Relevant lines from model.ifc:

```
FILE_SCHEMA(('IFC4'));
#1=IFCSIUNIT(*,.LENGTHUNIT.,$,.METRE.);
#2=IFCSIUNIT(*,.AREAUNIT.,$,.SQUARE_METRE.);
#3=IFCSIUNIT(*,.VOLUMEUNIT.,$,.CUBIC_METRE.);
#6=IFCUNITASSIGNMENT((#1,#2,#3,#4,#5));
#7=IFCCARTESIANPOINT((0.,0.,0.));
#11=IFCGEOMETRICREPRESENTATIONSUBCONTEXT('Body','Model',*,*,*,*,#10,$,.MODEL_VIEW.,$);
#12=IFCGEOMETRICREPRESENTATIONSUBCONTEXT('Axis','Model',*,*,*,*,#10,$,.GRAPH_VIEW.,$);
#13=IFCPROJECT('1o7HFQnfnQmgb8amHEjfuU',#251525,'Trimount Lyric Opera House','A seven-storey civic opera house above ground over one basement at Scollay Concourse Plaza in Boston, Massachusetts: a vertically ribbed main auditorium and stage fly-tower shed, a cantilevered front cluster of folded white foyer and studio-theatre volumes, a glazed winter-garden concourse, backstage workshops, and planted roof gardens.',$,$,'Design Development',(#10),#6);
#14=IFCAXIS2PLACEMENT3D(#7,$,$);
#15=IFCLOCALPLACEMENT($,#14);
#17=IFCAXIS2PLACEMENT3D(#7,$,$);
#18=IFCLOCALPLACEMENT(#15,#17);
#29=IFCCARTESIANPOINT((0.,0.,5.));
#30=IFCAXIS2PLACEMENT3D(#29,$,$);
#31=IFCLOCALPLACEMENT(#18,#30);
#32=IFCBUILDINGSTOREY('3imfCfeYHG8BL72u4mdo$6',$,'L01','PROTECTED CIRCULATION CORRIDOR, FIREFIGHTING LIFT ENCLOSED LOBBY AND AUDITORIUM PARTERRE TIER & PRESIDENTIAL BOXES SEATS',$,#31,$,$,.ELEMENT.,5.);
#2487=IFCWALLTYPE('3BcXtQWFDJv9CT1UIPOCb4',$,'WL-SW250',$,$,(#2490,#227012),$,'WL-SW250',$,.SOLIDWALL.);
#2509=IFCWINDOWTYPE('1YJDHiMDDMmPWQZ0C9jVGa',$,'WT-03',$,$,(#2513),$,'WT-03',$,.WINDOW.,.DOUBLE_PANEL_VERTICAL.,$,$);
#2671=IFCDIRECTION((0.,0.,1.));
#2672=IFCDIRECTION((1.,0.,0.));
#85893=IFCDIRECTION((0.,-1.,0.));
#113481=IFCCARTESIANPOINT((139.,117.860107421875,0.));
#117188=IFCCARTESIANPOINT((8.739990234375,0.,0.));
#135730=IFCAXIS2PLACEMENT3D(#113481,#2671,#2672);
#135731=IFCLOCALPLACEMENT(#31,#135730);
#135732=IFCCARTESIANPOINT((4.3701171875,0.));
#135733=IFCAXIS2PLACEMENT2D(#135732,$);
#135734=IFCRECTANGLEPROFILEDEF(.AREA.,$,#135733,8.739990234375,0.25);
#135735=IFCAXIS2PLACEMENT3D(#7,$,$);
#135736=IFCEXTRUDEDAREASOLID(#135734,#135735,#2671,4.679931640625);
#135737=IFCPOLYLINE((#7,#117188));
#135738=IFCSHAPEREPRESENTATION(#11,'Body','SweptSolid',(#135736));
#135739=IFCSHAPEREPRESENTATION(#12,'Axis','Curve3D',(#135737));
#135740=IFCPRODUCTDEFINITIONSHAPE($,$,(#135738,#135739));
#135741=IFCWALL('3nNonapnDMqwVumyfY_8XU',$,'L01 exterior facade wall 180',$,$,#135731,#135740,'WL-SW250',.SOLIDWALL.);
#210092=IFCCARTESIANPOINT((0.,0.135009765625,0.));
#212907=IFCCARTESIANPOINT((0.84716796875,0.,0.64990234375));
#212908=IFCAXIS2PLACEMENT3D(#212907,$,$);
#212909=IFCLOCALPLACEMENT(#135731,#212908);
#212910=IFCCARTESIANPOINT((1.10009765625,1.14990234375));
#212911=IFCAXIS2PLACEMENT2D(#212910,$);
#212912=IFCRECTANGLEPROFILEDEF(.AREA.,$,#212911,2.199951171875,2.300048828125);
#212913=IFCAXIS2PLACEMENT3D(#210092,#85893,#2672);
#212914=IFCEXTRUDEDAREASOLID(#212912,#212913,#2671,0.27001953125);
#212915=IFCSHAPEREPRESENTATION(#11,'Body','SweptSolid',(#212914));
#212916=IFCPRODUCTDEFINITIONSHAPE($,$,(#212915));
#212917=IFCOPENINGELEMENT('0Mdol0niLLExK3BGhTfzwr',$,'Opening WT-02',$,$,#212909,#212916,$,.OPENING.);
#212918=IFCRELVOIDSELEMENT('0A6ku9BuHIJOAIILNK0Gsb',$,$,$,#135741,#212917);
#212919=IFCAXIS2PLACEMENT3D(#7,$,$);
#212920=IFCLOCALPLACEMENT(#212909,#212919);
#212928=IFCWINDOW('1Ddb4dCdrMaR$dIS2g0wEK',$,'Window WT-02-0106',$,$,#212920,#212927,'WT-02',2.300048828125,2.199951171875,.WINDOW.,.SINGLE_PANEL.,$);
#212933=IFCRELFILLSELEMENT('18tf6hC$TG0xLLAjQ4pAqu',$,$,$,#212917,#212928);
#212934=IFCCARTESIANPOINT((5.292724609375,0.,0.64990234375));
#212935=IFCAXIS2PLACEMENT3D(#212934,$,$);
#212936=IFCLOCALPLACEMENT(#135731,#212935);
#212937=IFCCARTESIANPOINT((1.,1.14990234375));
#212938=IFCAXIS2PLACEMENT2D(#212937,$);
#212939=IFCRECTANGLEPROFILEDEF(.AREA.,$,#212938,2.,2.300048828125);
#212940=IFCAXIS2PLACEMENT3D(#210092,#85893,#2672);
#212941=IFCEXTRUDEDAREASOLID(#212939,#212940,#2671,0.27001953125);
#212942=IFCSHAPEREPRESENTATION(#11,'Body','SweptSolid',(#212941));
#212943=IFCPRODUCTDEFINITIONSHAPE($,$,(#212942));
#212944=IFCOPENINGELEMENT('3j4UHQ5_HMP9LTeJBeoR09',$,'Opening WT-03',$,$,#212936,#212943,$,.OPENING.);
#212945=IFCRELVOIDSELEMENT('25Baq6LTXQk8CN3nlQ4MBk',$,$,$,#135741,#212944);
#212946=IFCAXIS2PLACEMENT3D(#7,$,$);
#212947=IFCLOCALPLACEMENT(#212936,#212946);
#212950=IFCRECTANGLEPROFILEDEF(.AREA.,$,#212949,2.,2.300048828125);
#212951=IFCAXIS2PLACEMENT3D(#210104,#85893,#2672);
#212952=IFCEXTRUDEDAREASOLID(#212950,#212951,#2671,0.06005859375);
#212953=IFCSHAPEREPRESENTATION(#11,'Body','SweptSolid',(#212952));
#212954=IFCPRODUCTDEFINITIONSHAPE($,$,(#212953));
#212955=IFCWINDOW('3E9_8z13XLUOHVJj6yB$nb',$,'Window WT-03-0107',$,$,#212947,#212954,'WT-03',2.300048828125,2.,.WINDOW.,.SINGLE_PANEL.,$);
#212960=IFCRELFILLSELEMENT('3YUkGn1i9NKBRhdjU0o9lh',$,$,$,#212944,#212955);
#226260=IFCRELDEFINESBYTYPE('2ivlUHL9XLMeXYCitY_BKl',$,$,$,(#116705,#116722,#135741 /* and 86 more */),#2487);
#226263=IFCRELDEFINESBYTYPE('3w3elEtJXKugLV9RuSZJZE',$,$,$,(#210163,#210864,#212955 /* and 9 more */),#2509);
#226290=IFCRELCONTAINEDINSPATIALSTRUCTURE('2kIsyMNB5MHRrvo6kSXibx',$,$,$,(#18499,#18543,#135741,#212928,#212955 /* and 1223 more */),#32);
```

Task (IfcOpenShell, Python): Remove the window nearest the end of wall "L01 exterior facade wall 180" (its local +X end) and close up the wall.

```python
import ifcopenshell
import ifcopenshell.api.feature
import ifcopenshell.api.root
import ifcopenshell.geom
import ifcopenshell.util.shape

model = ifcopenshell.open("model.ifc")
settings = ifcopenshell.geom.settings()


def volume(element):
    """Net volume in cubic metres, openings subtracted."""
    shape = ifcopenshell.geom.create_shape(settings, element)
    return ifcopenshell.util.shape.get_volume(shape.geometry)


window = model.by_guid("3E9_8z13XLUOHVJj6yB$nb")
opening = window.FillsVoids[0].RelatingOpeningElement
wall = opening.VoidsElements[0].RelatingBuildingElement
before = volume(wall)

ifcopenshell.api.root.remove_product(model, product=window)
ifcopenshell.api.feature.remove_feature(model, feature=opening)

after = volume(wall)

print(f"wall volume {before:.3f} -> {after:.3f} m3")

model.write("model_updated.ifc")
```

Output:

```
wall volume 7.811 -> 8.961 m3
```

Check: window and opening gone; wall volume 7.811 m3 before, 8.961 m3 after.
